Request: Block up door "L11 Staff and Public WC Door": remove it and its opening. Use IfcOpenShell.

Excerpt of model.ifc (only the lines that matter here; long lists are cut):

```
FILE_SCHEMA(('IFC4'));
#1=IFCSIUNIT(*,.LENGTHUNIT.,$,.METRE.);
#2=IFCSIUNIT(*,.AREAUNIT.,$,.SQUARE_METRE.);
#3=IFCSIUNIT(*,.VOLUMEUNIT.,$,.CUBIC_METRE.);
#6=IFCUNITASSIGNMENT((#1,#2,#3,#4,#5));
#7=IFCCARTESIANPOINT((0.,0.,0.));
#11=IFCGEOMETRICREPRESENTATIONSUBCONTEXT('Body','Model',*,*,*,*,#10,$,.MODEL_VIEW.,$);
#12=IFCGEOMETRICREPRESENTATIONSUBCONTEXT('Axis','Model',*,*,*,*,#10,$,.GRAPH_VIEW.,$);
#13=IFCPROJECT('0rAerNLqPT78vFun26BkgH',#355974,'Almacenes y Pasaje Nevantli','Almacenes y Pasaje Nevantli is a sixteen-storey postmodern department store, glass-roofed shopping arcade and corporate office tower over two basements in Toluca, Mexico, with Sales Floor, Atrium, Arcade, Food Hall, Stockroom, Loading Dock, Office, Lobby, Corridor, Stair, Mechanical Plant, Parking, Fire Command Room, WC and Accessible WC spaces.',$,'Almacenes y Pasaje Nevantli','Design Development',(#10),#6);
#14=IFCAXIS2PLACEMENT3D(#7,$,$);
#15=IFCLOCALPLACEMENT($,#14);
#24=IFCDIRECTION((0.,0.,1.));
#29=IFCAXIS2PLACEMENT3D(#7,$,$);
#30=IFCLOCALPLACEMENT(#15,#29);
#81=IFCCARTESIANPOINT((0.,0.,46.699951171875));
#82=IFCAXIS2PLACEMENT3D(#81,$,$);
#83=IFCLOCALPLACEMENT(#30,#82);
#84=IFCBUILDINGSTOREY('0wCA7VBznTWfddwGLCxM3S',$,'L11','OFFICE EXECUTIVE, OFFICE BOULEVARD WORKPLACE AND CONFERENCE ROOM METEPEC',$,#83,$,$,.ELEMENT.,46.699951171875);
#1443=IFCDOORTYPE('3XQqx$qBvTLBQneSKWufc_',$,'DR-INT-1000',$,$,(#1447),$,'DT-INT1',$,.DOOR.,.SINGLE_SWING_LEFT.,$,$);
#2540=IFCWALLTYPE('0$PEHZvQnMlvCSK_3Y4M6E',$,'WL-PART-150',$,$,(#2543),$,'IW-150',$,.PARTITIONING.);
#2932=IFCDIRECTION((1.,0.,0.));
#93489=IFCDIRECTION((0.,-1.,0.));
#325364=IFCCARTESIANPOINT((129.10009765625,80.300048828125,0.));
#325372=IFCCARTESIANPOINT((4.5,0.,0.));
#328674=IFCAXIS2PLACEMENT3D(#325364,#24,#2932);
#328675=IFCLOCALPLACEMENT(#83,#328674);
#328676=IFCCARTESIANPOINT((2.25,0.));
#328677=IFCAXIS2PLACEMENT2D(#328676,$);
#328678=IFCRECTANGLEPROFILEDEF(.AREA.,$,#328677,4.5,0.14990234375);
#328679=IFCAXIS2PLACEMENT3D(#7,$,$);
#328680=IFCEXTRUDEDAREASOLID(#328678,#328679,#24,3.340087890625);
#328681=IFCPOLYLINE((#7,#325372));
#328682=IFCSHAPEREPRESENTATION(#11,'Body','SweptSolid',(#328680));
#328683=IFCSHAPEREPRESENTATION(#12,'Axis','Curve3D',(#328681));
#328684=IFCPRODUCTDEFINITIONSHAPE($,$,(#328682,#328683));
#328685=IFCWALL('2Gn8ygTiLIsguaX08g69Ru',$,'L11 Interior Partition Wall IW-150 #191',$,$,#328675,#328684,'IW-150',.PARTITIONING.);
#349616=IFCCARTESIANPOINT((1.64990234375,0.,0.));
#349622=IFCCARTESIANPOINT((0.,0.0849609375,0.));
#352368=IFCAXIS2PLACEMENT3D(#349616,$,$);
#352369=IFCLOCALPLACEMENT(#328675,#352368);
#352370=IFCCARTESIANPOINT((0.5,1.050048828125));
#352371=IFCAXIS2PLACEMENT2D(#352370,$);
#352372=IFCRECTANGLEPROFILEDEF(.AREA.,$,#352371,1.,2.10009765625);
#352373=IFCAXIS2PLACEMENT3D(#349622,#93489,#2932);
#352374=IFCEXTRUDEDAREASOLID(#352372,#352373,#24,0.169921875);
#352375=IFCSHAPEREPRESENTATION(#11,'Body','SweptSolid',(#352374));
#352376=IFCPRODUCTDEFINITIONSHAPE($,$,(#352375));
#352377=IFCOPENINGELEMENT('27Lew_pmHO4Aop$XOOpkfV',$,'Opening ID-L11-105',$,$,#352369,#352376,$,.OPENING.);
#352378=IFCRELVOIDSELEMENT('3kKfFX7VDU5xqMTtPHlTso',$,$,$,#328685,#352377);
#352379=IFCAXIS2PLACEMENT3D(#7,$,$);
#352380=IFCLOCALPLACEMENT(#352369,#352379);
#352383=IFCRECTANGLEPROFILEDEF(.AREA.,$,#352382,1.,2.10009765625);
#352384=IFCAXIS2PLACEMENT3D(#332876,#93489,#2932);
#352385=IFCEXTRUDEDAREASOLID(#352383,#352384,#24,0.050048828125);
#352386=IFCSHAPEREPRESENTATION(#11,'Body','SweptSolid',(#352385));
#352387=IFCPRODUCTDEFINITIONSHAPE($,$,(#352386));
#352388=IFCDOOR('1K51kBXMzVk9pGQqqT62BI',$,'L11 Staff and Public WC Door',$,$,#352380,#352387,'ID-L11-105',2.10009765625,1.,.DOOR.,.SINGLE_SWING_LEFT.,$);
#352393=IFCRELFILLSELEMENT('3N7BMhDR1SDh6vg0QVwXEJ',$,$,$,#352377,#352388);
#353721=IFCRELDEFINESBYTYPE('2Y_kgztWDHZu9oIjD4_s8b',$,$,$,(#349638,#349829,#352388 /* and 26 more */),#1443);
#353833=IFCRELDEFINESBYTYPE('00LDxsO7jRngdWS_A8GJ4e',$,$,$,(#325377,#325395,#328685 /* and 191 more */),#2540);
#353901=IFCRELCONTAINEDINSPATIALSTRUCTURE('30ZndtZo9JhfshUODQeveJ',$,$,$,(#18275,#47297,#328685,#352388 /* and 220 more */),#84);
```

```python
import ifcopenshell
import ifcopenshell.api.feature
import ifcopenshell.api.root
import ifcopenshell.geom
import ifcopenshell.util.shape

model = ifcopenshell.open("model.ifc")
settings = ifcopenshell.geom.settings()


def volume(element):
    """Net volume in cubic metres, openings subtracted."""
    shape = ifcopenshell.geom.create_shape(settings, element)
    return ifcopenshell.util.shape.get_volume(shape.geometry)


door = model.by_id(352388)
opening = door.FillsVoids[0].RelatingOpeningElement
wall = opening.VoidsElements[0].RelatingBuildingElement
before = volume(wall)

ifcopenshell.api.root.remove_product(model, product=door)
ifcopenshell.api.feature.remove_feature(model, feature=opening)

after = volume(wall)

print(f"wall volume {before:.3f} -> {after:.3f} m3")

model.write("model-out.ifc")
```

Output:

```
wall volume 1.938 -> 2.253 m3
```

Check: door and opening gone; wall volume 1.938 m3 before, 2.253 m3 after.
